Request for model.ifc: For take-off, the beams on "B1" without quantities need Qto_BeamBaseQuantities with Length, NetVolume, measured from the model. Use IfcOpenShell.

First a look at what the model holds.

```python
import ifcopenshell
import ifcopenshell.util.element
import ifcopenshell.util.unit

model = ifcopenshell.open("model.ifc")
print(model.schema)
for unit_type in ("LENGTHUNIT", "AREAUNIT", "VOLUMEUNIT"):
    print(unit_type, ifcopenshell.util.unit.calculate_unit_scale(model, unit_type))
storey = next(s for s in model.by_type("IfcBuildingStorey") if s.Name == "B1")
beams = [e for e in ifcopenshell.util.element.get_decomposition(storey) if e.is_a("IfcBeam")]
for e in sorted(beams, key=lambda e: e.id()):
    print(e.id(), e.is_a(), e.Name, list(ifcopenshell.util.element.get_psets(e, qtos_only=True)), sep=" | ")
```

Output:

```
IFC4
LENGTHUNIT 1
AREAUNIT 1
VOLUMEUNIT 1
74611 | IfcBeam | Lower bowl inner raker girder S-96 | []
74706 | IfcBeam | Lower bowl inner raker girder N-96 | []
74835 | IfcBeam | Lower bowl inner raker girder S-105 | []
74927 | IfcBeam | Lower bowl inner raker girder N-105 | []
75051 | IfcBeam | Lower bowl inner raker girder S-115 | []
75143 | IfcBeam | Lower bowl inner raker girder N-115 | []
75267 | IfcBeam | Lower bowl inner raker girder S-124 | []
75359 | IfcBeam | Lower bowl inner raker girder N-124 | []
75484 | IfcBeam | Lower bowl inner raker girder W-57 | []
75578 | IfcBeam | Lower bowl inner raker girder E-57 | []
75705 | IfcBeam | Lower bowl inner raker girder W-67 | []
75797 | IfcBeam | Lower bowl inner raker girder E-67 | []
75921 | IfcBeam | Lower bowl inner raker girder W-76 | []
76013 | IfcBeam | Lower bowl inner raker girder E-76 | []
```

```python
import ifcopenshell
import ifcopenshell.api.pset
import ifcopenshell.geom
import ifcopenshell.util.element
import ifcopenshell.util.shape
import ifcopenshell.util.unit

model = ifcopenshell.open("model.ifc")
unit_scale = ifcopenshell.util.unit.calculate_unit_scale(model)
volume_scale = ifcopenshell.util.unit.calculate_unit_scale(model, "VOLUMEUNIT")
settings = ifcopenshell.geom.settings()

storey = next(s for s in model.by_type("IfcBuildingStorey") if s.Name == "B1")
beams = [e for e in ifcopenshell.util.element.get_decomposition(storey) if e.is_a("IfcBeam")]

for e in sorted(beams, key=lambda e: e.id()):
    if ifcopenshell.util.element.get_psets(e, qtos_only=True, should_inherit=False):
        continue
    # Geometry comes back in metres, in the element's own axes.
    shape = ifcopenshell.geom.create_shape(settings, e)
    values = {
        "Length": ifcopenshell.util.shape.get_max_xyz(shape.geometry) / unit_scale,
        "NetVolume": ifcopenshell.util.shape.get_volume(shape.geometry) / volume_scale,
    }
    qto = ifcopenshell.api.pset.add_qto(model, product=e, name="Qto_BeamBaseQuantities")
    ifcopenshell.api.pset.edit_qto(model, qto=qto, properties=values)
    print(e.id(), {k: round(v, 3) for k, v in values.items()})

model.write("model_updated.ifc")
```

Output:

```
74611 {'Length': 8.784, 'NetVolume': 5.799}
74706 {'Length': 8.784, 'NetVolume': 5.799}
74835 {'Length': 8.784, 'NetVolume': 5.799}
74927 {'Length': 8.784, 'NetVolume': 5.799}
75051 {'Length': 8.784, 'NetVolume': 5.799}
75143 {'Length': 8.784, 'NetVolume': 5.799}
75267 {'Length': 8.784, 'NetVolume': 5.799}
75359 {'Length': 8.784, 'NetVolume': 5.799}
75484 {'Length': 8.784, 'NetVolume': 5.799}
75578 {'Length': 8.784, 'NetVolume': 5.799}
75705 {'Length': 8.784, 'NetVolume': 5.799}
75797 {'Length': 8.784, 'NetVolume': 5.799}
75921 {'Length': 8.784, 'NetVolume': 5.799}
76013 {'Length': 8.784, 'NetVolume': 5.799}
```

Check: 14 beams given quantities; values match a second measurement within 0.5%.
